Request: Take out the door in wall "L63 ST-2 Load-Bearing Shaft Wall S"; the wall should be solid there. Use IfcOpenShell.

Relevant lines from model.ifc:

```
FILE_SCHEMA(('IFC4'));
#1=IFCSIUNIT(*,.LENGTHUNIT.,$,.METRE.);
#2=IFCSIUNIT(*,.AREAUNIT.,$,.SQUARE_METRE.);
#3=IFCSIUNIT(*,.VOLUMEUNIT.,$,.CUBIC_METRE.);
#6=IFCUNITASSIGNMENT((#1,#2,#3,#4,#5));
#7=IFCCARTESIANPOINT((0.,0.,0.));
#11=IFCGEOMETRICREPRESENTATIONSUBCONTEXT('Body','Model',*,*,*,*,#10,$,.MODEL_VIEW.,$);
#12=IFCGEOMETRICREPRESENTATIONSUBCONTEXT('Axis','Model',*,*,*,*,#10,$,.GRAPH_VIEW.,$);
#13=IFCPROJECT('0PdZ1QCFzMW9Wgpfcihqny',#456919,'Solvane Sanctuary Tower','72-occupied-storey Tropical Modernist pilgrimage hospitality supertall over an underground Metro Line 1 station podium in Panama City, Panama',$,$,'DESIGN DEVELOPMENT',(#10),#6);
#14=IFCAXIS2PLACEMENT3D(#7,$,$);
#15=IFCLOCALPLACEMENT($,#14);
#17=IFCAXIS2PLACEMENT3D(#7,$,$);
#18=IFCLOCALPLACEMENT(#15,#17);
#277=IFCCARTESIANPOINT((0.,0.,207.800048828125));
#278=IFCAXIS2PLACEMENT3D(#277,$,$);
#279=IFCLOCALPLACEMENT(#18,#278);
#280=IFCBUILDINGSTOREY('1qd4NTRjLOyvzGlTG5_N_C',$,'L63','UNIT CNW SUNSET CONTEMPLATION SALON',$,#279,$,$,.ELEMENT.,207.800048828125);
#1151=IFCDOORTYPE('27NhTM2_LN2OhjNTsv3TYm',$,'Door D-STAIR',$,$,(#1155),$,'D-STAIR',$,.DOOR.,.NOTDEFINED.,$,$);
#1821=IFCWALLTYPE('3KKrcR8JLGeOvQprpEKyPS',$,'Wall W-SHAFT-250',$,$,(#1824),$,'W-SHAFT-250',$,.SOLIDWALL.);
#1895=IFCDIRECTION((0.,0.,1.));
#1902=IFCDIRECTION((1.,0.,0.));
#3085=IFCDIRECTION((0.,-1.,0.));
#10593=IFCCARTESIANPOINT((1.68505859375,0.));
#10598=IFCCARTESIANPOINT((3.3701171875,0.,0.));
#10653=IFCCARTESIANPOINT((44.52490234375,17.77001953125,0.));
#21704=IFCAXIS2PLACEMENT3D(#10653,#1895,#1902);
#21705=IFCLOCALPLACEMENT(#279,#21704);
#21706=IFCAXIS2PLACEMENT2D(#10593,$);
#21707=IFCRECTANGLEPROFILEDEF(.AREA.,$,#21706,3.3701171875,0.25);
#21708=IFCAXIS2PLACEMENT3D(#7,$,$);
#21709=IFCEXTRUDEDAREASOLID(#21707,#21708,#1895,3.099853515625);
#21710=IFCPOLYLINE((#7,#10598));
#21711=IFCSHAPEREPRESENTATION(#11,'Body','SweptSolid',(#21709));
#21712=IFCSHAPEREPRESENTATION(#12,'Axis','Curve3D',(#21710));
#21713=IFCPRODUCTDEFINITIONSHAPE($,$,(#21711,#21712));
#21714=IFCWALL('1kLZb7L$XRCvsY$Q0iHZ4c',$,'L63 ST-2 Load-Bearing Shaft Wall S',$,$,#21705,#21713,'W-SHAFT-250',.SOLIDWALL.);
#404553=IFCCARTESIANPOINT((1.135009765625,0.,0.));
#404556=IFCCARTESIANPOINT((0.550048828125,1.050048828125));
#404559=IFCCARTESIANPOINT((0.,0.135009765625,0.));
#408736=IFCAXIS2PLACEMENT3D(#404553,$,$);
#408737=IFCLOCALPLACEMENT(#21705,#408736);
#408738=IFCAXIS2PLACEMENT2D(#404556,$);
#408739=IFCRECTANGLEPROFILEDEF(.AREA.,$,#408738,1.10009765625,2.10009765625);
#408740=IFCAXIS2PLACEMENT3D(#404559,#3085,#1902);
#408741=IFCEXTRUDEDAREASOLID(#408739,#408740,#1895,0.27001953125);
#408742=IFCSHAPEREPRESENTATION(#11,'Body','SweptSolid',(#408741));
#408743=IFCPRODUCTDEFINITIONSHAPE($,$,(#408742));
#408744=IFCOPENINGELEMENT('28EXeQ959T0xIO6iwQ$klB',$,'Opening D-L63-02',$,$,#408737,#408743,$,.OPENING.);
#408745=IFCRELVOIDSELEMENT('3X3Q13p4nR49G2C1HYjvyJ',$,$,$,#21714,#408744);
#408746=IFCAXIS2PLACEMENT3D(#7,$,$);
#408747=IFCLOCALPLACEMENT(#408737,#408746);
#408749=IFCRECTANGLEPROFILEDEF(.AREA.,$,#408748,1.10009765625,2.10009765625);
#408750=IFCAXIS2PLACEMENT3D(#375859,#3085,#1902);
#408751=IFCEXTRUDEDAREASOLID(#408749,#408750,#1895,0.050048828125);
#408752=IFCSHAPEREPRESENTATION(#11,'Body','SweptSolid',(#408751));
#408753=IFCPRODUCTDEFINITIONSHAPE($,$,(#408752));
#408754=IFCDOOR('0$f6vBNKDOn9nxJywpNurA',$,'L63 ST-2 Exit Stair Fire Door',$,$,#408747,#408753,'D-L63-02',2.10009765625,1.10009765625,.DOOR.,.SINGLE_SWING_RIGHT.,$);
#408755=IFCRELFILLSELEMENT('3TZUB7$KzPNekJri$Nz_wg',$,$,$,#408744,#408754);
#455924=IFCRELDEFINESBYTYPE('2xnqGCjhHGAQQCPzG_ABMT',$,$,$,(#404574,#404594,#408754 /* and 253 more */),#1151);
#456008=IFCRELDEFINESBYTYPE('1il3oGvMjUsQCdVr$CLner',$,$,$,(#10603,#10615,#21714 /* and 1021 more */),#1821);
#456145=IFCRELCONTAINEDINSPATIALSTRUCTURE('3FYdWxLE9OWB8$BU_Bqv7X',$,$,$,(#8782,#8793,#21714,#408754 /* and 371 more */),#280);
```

```python
import ifcopenshell
import ifcopenshell.api.feature
import ifcopenshell.api.root
import ifcopenshell.geom
import ifcopenshell.util.shape

model = ifcopenshell.open("model.ifc")
settings = ifcopenshell.geom.settings()


def volume(element):
    """Net volume in cubic metres, openings subtracted."""
    shape = ifcopenshell.geom.create_shape(settings, element)
    return ifcopenshell.util.shape.get_volume(shape.geometry)


door = model.by_guid("0$f6vBNKDOn9nxJywpNurA")
opening = door.FillsVoids[0].RelatingOpeningElement
wall = opening.VoidsElements[0].RelatingBuildingElement
before = volume(wall)

ifcopenshell.api.root.remove_product(model, product=door)
ifcopenshell.api.feature.remove_feature(model, feature=opening)

after = volume(wall)

print(f"wall volume {before:.3f} -> {after:.3f} m3")

model.write("model-out.ifc")
```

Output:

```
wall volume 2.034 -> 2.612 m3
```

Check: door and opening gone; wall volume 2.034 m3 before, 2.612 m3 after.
